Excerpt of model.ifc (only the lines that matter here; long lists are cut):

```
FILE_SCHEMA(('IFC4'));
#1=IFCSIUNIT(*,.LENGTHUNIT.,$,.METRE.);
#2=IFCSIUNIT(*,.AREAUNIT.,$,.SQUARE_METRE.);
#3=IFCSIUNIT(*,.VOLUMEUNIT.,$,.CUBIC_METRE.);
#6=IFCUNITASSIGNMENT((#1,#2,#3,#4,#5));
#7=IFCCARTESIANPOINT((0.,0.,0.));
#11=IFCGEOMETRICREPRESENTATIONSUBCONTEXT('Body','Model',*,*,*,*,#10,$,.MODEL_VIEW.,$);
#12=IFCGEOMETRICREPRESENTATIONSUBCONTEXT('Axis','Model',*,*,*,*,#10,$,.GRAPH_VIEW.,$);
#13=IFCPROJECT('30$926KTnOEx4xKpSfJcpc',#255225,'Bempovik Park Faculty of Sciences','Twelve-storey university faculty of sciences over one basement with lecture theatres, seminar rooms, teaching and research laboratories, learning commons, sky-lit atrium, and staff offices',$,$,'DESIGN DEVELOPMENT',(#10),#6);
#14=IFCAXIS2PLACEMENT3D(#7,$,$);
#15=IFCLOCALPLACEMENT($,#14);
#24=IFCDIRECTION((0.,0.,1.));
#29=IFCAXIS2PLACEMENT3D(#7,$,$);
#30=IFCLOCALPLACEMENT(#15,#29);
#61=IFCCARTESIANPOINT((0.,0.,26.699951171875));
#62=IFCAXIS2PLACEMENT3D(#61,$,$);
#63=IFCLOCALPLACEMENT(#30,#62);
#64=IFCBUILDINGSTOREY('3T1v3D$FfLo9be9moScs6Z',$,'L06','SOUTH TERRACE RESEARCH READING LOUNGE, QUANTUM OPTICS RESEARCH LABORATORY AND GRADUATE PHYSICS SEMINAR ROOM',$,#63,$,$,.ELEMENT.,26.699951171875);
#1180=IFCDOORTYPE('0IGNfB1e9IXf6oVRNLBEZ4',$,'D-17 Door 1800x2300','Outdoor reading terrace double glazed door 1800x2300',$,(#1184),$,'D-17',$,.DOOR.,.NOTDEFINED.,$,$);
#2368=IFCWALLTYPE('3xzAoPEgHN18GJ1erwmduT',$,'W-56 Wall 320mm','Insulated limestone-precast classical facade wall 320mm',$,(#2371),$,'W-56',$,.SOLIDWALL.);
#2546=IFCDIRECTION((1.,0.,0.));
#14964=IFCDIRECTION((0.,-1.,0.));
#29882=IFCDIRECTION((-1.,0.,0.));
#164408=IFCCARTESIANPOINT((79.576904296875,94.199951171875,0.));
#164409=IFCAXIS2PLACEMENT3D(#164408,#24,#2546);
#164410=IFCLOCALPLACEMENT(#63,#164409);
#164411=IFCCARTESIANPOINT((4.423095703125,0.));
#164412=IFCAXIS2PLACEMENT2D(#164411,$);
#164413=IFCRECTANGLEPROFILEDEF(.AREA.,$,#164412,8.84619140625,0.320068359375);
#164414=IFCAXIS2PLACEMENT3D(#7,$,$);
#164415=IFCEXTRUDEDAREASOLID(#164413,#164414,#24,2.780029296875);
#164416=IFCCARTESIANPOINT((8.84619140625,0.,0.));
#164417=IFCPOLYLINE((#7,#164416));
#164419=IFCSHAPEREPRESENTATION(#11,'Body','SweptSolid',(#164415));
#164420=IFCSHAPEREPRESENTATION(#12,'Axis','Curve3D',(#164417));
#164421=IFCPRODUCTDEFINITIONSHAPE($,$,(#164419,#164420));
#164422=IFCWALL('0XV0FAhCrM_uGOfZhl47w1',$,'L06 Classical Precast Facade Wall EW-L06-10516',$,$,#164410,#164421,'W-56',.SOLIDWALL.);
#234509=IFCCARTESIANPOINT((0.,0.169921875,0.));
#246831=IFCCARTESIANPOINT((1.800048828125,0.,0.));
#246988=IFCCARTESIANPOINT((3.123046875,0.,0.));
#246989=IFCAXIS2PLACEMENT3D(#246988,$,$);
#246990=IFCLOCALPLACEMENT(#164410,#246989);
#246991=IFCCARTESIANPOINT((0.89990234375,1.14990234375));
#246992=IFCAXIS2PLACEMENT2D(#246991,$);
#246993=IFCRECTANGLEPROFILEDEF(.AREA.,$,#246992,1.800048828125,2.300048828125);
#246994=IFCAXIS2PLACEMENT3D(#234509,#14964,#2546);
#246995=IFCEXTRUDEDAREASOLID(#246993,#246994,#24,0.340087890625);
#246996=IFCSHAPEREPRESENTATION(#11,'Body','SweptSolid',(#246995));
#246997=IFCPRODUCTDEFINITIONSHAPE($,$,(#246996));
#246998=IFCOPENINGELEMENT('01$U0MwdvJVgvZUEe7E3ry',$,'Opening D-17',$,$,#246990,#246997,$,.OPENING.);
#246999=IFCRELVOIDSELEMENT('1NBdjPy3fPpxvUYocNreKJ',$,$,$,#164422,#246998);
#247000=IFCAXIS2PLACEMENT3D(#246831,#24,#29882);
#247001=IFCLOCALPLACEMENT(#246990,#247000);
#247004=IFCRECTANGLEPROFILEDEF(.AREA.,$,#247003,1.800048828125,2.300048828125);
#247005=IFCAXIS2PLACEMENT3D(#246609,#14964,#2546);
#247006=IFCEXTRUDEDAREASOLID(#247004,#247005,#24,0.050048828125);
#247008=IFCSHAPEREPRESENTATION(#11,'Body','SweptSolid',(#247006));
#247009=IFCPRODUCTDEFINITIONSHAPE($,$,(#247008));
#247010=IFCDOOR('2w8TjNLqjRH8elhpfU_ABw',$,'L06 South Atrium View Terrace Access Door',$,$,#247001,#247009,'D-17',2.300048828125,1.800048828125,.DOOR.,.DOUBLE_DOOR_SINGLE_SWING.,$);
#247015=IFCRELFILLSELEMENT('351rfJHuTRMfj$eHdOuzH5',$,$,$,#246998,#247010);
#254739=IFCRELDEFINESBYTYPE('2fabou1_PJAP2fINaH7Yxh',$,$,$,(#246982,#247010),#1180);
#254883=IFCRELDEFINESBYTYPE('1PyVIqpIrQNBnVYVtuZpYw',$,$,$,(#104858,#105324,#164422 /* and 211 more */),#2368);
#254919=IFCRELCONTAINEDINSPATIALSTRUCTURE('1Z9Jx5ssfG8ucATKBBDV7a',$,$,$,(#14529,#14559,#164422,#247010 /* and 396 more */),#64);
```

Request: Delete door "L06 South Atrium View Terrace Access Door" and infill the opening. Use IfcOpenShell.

```python
import ifcopenshell
import ifcopenshell.api.feature
import ifcopenshell.api.root
import ifcopenshell.geom
import ifcopenshell.util.shape

model = ifcopenshell.open("model.ifc")
settings = ifcopenshell.geom.settings()


def volume(element):
    """Net volume in cubic metres, openings subtracted."""
    shape = ifcopenshell.geom.create_shape(settings, element)
    return ifcopenshell.util.shape.get_volume(shape.geometry)


door = model.by_id(247010)
opening = door.FillsVoids[0].RelatingOpeningElement
wall = opening.VoidsElements[0].RelatingBuildingElement
before = volume(wall)

ifcopenshell.api.root.remove_product(model, product=door)
ifcopenshell.api.feature.remove_feature(model, feature=opening)

after = volume(wall)

print(f"wall volume {before:.3f} -> {after:.3f} m3")

model.write("model-out.ifc")
```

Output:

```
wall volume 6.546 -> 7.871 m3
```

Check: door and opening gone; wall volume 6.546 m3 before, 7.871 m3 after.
